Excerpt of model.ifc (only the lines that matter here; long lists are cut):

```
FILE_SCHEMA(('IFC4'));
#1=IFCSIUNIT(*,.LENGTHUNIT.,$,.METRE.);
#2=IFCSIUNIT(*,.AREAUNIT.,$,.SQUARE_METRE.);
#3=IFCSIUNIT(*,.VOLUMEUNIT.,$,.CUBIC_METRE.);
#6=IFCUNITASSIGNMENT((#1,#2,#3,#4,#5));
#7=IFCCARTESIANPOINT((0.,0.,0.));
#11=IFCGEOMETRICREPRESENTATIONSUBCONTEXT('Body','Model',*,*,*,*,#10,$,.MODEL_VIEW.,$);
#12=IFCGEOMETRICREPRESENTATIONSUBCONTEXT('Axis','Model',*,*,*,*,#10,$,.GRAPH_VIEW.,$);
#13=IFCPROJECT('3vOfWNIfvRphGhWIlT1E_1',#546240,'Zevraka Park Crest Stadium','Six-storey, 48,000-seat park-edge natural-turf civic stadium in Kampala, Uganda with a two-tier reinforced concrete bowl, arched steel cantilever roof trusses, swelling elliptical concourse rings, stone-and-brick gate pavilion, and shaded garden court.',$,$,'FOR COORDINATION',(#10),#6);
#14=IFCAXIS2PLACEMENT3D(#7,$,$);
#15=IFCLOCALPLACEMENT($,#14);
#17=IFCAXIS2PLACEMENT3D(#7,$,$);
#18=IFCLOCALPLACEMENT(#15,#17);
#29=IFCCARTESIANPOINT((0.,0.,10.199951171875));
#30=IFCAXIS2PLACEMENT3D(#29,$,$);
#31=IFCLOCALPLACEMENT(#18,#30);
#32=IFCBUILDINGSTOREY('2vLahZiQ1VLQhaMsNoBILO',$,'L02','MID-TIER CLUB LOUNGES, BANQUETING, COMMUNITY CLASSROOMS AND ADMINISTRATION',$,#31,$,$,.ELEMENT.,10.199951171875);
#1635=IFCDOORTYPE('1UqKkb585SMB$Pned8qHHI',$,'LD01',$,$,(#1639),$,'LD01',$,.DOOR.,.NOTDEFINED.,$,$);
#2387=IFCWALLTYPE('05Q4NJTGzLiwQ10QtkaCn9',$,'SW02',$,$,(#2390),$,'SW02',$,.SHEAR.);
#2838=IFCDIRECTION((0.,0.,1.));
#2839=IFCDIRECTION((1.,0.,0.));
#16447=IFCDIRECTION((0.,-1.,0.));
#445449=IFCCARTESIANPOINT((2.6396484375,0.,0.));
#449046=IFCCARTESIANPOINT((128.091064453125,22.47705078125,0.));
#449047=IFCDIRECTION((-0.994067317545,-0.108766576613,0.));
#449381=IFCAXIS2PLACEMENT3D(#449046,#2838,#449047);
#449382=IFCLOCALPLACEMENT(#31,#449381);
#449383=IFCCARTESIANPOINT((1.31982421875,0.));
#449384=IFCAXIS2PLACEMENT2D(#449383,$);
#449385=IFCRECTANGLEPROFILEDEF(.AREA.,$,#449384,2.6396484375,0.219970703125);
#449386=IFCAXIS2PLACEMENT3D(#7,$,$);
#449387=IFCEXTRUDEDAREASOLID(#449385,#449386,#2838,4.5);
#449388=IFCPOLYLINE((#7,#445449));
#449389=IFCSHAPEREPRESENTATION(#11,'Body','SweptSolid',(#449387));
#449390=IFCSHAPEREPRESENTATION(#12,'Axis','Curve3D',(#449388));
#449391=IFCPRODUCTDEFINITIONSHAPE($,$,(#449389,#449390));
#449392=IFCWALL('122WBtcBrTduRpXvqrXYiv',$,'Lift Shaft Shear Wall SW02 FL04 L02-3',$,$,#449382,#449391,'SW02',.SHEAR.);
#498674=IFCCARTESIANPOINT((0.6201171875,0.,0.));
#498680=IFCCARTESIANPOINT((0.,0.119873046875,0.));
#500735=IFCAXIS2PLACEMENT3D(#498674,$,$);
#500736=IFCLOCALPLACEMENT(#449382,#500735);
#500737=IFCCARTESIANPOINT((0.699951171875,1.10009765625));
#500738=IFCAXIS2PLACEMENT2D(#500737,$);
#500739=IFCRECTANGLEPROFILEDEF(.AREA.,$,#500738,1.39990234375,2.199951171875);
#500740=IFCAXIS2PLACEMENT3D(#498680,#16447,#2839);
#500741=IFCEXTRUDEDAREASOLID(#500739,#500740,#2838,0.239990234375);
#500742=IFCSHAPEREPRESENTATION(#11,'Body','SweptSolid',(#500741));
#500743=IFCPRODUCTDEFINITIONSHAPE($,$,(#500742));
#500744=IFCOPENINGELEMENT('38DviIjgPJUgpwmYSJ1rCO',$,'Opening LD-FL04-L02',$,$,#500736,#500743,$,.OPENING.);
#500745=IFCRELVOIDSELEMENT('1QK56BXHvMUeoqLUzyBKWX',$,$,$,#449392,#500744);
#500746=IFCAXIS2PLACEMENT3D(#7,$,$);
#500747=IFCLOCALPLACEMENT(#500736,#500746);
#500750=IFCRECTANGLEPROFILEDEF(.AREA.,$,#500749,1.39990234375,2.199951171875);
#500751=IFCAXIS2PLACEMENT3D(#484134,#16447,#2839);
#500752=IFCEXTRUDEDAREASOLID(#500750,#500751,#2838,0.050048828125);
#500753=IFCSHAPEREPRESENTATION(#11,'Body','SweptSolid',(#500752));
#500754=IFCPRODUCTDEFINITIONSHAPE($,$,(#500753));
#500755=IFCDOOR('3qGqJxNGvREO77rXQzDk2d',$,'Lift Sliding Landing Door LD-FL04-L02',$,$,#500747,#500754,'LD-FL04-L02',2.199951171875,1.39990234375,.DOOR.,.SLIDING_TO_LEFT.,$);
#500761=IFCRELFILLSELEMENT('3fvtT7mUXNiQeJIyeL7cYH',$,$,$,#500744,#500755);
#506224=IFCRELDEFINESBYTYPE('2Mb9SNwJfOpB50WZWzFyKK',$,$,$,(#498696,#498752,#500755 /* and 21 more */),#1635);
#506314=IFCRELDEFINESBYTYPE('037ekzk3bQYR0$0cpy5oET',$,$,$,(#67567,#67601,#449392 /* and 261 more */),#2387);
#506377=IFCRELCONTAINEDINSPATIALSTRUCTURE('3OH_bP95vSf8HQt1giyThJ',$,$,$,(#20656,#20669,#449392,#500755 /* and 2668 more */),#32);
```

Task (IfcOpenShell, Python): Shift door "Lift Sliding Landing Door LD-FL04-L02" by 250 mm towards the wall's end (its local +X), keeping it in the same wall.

```python
import ifcopenshell
import ifcopenshell.api.geometry
import ifcopenshell.util.placement
import ifcopenshell.util.unit

model = ifcopenshell.open("model.ifc")
unit_scale = ifcopenshell.util.unit.calculate_unit_scale(model)

door = model.by_id(500755)
opening = door.FillsVoids[0].RelatingOpeningElement
wall = opening.VoidsElements[0].RelatingBuildingElement

wall_matrix = ifcopenshell.util.placement.get_local_placement(wall.ObjectPlacement)
shift = wall_matrix[:3, 0] * 0.25 / unit_scale
before = ifcopenshell.util.placement.get_local_placement(door.ObjectPlacement)[:3, 3].copy()

# The door is placed relative to its opening, so it follows when the opening moves.
matrix = ifcopenshell.util.placement.get_local_placement(opening.ObjectPlacement)
matrix[:3, 3] += shift
ifcopenshell.api.geometry.edit_object_placement(
    model, product=opening, matrix=matrix, is_si=False, should_transform_children=True
)

after = ifcopenshell.util.placement.get_local_placement(door.ObjectPlacement)[:3, 3]
print("door moved by", (after - before).round(3) + 0.0)

model.write("model_edited.ifc")
```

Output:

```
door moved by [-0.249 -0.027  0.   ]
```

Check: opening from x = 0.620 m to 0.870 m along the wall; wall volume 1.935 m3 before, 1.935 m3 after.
